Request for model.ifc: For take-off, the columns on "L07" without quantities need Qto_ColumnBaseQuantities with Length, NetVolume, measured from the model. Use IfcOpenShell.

First a look at what the model holds.

```python
import ifcopenshell
import ifcopenshell.util.element
import ifcopenshell.util.unit

model = ifcopenshell.open("model.ifc")
print(model.schema)
for unit_type in ("LENGTHUNIT", "AREAUNIT", "VOLUMEUNIT"):
    print(unit_type, ifcopenshell.util.unit.calculate_unit_scale(model, unit_type))
storey = next(s for s in model.by_type("IfcBuildingStorey") if s.Name == "L07")
columns = [e for e in ifcopenshell.util.element.get_decomposition(storey) if e.is_a("IfcColumn")]
for e in sorted(columns, key=lambda e: e.id()):
    print(e.id(), e.is_a(), e.Name, list(ifcopenshell.util.element.get_psets(e, qtos_only=True)), sep=" | ")
```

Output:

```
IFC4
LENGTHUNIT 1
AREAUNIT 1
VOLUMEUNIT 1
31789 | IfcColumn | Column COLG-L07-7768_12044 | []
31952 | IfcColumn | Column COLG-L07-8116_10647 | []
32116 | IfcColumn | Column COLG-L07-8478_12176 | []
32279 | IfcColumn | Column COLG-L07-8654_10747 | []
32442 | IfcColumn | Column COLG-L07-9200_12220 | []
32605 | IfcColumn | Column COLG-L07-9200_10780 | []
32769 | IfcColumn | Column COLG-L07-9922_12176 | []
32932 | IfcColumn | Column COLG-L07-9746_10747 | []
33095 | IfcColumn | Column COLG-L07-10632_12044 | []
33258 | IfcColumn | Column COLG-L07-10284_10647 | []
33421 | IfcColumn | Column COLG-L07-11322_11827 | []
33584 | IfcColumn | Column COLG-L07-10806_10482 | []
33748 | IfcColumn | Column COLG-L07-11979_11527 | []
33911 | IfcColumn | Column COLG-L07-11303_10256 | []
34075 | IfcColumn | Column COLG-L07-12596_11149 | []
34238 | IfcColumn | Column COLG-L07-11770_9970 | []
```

```python
import ifcopenshell
import ifcopenshell.api.pset
import ifcopenshell.geom
import ifcopenshell.util.element
import ifcopenshell.util.shape
import ifcopenshell.util.unit

model = ifcopenshell.open("model.ifc")
unit_scale = ifcopenshell.util.unit.calculate_unit_scale(model)
volume_scale = ifcopenshell.util.unit.calculate_unit_scale(model, "VOLUMEUNIT")
settings = ifcopenshell.geom.settings()

storey = next(s for s in model.by_type("IfcBuildingStorey") if s.Name == "L07")
columns = [e for e in ifcopenshell.util.element.get_decomposition(storey) if e.is_a("IfcColumn")]

for e in sorted(columns, key=lambda e: e.id()):
    if ifcopenshell.util.element.get_psets(e, qtos_only=True, should_inherit=False):
        continue
    # Geometry comes back in metres, in the element's own axes.
    shape = ifcopenshell.geom.create_shape(settings, e)
    values = {
        "Length": ifcopenshell.util.shape.get_z(shape.geometry) / unit_scale,
        "NetVolume": ifcopenshell.util.shape.get_volume(shape.geometry) / volume_scale,
    }
    qto = ifcopenshell.api.pset.add_qto(model, product=e, name="Qto_ColumnBaseQuantities")
    ifcopenshell.api.pset.edit_qto(model, qto=qto, properties=values)
    print(e.id(), {k: round(v, 3) for k, v in values.items()})

model.write("model_edited.ifc")
```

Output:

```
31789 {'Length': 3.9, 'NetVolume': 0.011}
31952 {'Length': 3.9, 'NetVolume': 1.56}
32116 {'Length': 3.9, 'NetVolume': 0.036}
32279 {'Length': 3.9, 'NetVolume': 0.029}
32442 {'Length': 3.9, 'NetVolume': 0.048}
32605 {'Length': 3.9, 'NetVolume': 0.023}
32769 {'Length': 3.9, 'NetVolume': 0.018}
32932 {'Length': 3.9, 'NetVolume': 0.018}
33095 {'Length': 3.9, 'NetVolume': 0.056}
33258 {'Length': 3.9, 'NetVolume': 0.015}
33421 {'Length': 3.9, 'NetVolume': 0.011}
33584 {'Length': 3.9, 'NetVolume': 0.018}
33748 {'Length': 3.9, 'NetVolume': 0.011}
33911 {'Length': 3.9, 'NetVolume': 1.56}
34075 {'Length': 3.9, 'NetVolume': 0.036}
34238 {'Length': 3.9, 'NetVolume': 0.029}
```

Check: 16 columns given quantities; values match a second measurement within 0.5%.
